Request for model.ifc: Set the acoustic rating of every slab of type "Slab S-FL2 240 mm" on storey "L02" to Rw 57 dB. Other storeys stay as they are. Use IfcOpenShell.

First a look at what the model holds.

```python
import ifcopenshell
import ifcopenshell.util.element

model = ifcopenshell.open("model.ifc")
print(model.schema)
storey = next(s for s in model.by_type("IfcBuildingStorey") if s.Name == "L02")
slabs = [e for e in ifcopenshell.util.element.get_decomposition(storey) if e.is_a("IfcSlab")]
seen = {}
for e in slabs:
    element_type = ifcopenshell.util.element.get_type(e)
    key = (element_type.Name if element_type != e and element_type else None, ifcopenshell.util.element.get_pset(e, "Pset_SlabCommon", "AcousticRating"))
    seen[key] = seen.get(key, 0) + 1
for (name, value), count in sorted(seen.items(), key=str):
    print(count, "x", name, "|", value)
```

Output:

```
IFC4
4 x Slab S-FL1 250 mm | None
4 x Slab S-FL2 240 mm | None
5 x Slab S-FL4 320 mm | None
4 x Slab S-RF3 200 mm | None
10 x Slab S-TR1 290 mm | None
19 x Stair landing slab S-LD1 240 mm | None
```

```python
import ifcopenshell
import ifcopenshell.api.pset
import ifcopenshell.util.element

model = ifcopenshell.open("model.ifc")

storey = next(s for s in model.by_type("IfcBuildingStorey") if s.Name == "L02")
slabs = [e for e in ifcopenshell.util.element.get_decomposition(storey) if e.is_a("IfcSlab")]

count = 0
for e in slabs:
    element_type = ifcopenshell.util.element.get_type(e)
    if element_type in (None, e) or element_type.Name != "Slab S-FL2 240 mm":
        continue
    # add_pset returns the element's existing set when there is one.
    pset = ifcopenshell.api.pset.add_pset(model, product=e, name="Pset_SlabCommon")
    ifcopenshell.api.pset.edit_pset(model, pset=pset, properties={"AcousticRating": "Rw 57 dB"})
    count += 1

print(count, "slabs updated")

model.write("model_v2.ifc")
```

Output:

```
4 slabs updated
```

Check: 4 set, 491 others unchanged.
